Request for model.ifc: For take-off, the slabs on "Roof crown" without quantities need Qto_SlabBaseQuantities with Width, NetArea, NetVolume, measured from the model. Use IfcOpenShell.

First a look at what the model holds.

```python
import ifcopenshell
import ifcopenshell.util.element
import ifcopenshell.util.unit

model = ifcopenshell.open("model.ifc")
print(model.schema)
for unit_type in ("LENGTHUNIT", "AREAUNIT", "VOLUMEUNIT"):
    print(unit_type, ifcopenshell.util.unit.calculate_unit_scale(model, unit_type))
storey = next(s for s in model.by_type("IfcBuildingStorey") if s.Name == "Roof crown")
slabs = [e for e in ifcopenshell.util.element.get_decomposition(storey) if e.is_a("IfcSlab")]
for e in sorted(slabs, key=lambda e: e.id()):
    print(e.id(), e.is_a(), e.Name, list(ifcopenshell.util.element.get_psets(e, qtos_only=True)), sep=" | ")
```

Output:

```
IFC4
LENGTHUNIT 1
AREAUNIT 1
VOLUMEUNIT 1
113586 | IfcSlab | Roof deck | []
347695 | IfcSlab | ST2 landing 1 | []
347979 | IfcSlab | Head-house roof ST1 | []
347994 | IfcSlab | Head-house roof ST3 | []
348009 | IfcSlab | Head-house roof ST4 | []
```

```python
import ifcopenshell
import ifcopenshell.api.pset
import ifcopenshell.geom
import ifcopenshell.util.element
import ifcopenshell.util.shape
import ifcopenshell.util.unit

model = ifcopenshell.open("model.ifc")
unit_scale = ifcopenshell.util.unit.calculate_unit_scale(model)
area_scale = ifcopenshell.util.unit.calculate_unit_scale(model, "AREAUNIT")
volume_scale = ifcopenshell.util.unit.calculate_unit_scale(model, "VOLUMEUNIT")
settings = ifcopenshell.geom.settings()

storey = next(s for s in model.by_type("IfcBuildingStorey") if s.Name == "Roof crown")
slabs = [e for e in ifcopenshell.util.element.get_decomposition(storey) if e.is_a("IfcSlab")]

for e in sorted(slabs, key=lambda e: e.id()):
    if ifcopenshell.util.element.get_psets(e, qtos_only=True, should_inherit=False):
        continue
    # Geometry comes back in metres, in the element's own axes.
    shape = ifcopenshell.geom.create_shape(settings, e)
    values = {
        "Width": ifcopenshell.util.shape.get_z(shape.geometry) / unit_scale,
        "NetArea": ifcopenshell.util.shape.get_footprint_area(shape.geometry) / area_scale,
        "NetVolume": ifcopenshell.util.shape.get_volume(shape.geometry) / volume_scale,
    }
    qto = ifcopenshell.api.pset.add_qto(model, product=e, name="Qto_SlabBaseQuantities")
    ifcopenshell.api.pset.edit_qto(model, qto=qto, properties=values)
    print(e.id(), {k: round(v, 3) for k, v in values.items()})

model.write("model-out.ifc")
```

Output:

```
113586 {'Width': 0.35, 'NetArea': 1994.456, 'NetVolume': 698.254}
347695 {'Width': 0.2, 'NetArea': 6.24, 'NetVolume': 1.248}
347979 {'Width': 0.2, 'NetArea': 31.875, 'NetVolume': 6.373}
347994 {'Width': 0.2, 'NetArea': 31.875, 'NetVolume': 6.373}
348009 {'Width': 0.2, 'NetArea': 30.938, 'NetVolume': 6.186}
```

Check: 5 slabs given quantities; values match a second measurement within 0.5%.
